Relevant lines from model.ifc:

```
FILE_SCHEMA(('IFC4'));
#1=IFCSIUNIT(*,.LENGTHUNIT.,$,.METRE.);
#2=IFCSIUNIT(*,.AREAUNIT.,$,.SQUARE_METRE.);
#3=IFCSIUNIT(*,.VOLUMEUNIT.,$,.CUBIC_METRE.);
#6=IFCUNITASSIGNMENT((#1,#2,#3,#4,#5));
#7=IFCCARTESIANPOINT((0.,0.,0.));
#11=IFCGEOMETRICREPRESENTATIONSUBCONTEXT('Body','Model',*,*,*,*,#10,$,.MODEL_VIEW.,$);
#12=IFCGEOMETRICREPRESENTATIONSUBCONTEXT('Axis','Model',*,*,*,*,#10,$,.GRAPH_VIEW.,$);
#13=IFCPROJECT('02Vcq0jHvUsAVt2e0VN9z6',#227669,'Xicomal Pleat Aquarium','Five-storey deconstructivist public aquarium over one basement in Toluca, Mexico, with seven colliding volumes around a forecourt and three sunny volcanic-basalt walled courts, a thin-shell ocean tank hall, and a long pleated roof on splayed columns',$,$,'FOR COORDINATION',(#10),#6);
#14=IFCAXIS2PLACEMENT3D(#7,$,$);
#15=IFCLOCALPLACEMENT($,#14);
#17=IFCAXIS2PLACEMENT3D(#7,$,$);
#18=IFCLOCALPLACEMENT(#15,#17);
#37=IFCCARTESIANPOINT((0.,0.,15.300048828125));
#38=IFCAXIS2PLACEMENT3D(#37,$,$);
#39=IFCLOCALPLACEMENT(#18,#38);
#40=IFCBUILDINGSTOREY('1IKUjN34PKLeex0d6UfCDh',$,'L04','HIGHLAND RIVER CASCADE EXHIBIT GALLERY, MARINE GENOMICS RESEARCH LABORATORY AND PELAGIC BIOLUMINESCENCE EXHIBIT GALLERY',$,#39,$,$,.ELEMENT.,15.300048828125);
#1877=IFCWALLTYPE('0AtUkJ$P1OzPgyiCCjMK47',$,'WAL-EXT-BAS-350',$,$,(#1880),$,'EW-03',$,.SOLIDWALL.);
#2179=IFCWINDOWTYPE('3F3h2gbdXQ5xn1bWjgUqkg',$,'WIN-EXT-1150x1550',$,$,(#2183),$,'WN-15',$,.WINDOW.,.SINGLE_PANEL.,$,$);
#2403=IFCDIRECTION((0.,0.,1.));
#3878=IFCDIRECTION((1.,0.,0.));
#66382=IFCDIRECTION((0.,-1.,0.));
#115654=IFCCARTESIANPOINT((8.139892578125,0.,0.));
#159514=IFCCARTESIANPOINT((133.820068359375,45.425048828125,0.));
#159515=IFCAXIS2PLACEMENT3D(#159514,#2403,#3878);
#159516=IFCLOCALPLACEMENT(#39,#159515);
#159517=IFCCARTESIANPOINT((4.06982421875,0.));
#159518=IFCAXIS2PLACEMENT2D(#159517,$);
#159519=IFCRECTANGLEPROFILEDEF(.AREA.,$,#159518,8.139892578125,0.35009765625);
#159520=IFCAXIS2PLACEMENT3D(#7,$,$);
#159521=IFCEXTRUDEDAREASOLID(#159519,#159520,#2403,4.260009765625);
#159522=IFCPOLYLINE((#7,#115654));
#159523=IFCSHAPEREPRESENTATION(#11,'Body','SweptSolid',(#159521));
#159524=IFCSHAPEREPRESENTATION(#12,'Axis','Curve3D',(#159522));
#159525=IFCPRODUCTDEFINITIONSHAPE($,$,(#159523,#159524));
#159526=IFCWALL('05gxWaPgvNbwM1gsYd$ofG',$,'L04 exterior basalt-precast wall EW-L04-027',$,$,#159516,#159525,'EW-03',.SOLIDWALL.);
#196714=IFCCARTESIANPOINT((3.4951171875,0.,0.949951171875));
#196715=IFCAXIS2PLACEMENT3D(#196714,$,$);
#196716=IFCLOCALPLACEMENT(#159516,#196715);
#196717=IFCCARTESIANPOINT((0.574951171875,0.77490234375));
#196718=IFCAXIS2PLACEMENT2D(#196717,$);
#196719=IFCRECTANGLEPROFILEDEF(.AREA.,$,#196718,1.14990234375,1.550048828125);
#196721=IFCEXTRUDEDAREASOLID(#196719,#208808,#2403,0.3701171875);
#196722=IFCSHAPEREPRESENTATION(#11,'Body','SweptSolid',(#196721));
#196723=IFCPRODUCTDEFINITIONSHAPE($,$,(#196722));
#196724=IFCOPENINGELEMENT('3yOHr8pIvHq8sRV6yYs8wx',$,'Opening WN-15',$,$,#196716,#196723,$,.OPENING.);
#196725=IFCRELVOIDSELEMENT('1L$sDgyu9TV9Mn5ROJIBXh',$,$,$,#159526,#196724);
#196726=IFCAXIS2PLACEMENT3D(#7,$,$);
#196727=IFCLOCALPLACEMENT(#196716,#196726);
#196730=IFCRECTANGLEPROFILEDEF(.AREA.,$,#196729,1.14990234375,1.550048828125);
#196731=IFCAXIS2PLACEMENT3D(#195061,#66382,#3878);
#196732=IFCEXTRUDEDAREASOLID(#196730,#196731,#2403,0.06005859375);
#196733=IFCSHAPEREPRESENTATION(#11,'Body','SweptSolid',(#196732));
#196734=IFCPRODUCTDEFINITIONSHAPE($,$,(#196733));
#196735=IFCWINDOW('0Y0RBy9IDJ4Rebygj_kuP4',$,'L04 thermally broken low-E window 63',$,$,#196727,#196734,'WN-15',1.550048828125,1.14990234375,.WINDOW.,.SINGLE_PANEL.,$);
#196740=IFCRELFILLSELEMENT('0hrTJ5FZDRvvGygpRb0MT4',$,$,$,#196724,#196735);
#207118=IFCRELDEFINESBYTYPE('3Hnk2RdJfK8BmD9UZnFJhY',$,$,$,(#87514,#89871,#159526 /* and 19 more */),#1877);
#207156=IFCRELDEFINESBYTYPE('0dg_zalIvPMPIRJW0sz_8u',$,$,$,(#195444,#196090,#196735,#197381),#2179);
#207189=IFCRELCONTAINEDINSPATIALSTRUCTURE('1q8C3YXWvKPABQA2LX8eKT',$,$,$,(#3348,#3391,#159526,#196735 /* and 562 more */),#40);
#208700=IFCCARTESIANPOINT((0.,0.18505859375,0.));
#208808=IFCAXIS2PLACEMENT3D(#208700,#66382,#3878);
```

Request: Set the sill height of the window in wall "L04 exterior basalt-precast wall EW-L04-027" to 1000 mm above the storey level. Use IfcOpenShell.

```python
import numpy as np
import ifcopenshell
import ifcopenshell.api.geometry
import ifcopenshell.geom
import ifcopenshell.util.element
import ifcopenshell.util.placement
import ifcopenshell.util.shape
import ifcopenshell.util.unit

model = ifcopenshell.open("model.ifc")
unit_scale = ifcopenshell.util.unit.calculate_unit_scale(model)

window = model.by_guid("0Y0RBy9IDJ4Rebygj_kuP4")
opening = window.FillsVoids[0].RelatingOpeningElement
storey = ifcopenshell.util.element.get_container(window, ifc_class="IfcBuildingStorey")
level = ifcopenshell.util.placement.get_local_placement(storey.ObjectPlacement)[2, 3]

# The opening's origin need not be at the sill, so measure its lowest point.
shape = ifcopenshell.geom.create_shape(ifcopenshell.geom.settings(), opening)
bottom = ifcopenshell.util.shape.get_shape_bottom_elevation(shape, shape.geometry) / unit_scale
dz = level + 1 / unit_scale - bottom

shift = np.array([0.0, 0.0, dz])
# The window is placed relative to its opening, so it follows when the opening moves.
matrix = ifcopenshell.util.placement.get_local_placement(opening.ObjectPlacement)
matrix[:3, 3] += shift
ifcopenshell.api.geometry.edit_object_placement(
    model, product=opening, matrix=matrix, is_si=False, should_transform_children=True
)

print(f"moved by {dz * unit_scale:+.3f} m")

model.write("model_v2.ifc")
```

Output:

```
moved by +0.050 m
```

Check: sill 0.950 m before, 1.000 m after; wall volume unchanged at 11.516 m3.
